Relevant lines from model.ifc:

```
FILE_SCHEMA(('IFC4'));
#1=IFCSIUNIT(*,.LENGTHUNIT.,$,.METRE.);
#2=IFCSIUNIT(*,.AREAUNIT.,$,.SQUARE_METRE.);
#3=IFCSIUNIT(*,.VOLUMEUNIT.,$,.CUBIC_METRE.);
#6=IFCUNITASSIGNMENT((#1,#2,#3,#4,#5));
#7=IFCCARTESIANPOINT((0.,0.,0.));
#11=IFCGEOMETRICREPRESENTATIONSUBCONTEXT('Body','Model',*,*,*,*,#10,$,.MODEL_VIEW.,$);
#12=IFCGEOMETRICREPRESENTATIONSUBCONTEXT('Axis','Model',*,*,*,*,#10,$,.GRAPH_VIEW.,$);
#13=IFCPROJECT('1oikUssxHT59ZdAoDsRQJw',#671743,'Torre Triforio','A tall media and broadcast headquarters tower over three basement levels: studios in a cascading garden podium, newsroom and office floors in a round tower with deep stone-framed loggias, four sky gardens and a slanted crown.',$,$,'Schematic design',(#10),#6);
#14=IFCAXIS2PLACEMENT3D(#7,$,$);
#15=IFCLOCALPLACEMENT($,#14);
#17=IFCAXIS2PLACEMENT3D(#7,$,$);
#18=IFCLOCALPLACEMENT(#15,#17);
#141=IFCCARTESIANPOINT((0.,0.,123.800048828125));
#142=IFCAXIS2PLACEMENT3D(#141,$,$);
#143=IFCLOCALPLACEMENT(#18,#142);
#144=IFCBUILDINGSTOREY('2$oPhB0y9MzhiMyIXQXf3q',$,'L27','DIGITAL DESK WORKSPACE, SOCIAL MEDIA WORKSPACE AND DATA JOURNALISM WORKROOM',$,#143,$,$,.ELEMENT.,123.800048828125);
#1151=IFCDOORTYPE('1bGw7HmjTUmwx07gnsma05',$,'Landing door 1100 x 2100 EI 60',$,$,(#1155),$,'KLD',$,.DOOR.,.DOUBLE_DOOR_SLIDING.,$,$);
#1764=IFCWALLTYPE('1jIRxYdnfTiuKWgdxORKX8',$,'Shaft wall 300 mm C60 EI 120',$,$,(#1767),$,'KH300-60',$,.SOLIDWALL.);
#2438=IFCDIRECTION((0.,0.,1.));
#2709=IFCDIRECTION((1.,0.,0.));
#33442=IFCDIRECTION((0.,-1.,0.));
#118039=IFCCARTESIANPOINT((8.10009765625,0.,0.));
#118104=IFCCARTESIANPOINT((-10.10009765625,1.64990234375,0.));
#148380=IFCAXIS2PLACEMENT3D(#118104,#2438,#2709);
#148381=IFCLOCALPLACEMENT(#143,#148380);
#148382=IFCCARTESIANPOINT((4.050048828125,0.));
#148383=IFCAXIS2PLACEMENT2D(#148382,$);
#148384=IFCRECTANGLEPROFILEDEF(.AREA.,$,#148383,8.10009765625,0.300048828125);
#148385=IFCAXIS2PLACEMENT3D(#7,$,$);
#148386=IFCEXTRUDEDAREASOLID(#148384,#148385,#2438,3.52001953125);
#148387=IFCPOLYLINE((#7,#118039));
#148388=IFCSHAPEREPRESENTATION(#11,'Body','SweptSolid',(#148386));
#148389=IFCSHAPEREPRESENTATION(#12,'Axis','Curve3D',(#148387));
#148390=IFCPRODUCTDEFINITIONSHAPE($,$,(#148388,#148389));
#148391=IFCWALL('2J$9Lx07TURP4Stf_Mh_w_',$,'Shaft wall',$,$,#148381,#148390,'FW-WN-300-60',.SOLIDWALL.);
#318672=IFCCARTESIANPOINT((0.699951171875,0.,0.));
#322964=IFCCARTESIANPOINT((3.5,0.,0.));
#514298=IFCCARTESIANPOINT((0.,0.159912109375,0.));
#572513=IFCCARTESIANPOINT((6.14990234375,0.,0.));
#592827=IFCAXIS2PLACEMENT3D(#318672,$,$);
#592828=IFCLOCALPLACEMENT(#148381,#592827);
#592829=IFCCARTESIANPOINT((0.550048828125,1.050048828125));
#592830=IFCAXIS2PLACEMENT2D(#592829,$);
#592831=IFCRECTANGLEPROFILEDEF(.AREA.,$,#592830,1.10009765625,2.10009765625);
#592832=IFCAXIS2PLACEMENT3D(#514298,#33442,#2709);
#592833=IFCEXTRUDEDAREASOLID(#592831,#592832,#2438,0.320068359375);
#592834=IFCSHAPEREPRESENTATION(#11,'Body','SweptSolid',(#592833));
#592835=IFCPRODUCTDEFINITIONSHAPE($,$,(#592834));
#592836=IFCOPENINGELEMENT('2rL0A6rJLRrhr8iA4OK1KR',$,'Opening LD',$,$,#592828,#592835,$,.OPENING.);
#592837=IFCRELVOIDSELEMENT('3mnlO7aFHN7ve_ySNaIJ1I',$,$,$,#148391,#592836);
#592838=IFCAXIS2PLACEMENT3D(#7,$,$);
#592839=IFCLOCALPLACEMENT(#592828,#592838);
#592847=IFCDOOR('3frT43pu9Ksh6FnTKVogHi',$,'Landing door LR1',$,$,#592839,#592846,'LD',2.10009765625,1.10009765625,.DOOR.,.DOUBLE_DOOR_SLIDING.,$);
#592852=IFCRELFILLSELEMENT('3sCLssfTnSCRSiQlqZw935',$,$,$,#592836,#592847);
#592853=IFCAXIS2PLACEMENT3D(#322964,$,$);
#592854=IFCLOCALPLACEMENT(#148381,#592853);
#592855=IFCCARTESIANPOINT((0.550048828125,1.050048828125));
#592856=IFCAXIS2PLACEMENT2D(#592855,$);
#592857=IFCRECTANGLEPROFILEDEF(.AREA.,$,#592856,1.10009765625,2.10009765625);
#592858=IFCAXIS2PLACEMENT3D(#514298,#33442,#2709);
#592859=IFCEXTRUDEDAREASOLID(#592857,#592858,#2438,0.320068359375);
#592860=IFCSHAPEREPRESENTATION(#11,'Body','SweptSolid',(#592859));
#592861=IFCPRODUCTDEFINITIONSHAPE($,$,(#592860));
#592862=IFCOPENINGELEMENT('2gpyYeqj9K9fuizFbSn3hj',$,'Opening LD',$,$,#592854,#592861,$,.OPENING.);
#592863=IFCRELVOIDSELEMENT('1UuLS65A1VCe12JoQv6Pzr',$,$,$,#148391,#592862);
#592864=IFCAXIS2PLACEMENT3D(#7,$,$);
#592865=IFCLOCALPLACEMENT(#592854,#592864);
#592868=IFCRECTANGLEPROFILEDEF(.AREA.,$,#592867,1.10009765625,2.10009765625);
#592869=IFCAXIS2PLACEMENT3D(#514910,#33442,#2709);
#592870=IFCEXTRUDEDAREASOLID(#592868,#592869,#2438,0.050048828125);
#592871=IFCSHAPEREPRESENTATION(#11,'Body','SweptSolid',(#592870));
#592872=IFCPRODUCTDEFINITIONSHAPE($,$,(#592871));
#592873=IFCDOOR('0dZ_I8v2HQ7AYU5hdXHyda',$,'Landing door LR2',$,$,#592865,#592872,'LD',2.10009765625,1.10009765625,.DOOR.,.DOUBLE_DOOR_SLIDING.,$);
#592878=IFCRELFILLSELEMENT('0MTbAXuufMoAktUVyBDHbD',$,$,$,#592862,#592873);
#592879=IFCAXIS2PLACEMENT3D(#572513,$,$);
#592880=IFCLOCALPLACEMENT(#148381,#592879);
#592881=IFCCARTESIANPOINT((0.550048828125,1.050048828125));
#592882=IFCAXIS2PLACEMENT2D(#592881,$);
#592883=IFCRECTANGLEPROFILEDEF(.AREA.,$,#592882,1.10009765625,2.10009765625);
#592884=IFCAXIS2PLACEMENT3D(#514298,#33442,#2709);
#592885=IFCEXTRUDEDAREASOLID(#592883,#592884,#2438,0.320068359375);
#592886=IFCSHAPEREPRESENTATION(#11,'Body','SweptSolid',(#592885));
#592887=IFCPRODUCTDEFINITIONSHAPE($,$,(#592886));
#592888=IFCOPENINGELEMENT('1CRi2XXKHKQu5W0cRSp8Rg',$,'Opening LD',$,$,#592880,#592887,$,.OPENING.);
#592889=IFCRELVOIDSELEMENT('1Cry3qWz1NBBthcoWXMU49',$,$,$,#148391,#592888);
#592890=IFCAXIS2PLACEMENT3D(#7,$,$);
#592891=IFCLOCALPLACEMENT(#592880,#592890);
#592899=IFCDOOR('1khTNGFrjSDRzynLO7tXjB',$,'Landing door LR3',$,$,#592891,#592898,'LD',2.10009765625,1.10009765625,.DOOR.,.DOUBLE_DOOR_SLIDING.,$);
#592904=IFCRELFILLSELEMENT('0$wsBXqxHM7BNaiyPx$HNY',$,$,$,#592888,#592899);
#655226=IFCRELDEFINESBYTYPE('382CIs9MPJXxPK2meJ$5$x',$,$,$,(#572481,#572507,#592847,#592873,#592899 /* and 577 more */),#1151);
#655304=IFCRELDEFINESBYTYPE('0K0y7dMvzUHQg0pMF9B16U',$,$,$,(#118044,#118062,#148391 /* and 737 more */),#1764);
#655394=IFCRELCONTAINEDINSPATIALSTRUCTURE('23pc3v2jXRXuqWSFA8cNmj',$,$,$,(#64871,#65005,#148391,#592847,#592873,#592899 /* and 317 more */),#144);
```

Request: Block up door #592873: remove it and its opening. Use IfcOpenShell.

```python
import ifcopenshell
import ifcopenshell.api.feature
import ifcopenshell.api.root
import ifcopenshell.geom
import ifcopenshell.util.shape

model = ifcopenshell.open("model.ifc")
settings = ifcopenshell.geom.settings()


def volume(element):
    """Net volume in cubic metres, openings subtracted."""
    shape = ifcopenshell.geom.create_shape(settings, element)
    return ifcopenshell.util.shape.get_volume(shape.geometry)


door = model.by_guid("0dZ_I8v2HQ7AYU5hdXHyda")
opening = door.FillsVoids[0].RelatingOpeningElement
wall = opening.VoidsElements[0].RelatingBuildingElement
before = volume(wall)

ifcopenshell.api.root.remove_product(model, product=door)
ifcopenshell.api.feature.remove_feature(model, feature=opening)

after = volume(wall)

print(f"wall volume {before:.3f} -> {after:.3f} m3")

model.write("model-out.ifc")
```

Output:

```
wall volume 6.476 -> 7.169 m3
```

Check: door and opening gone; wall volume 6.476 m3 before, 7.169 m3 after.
